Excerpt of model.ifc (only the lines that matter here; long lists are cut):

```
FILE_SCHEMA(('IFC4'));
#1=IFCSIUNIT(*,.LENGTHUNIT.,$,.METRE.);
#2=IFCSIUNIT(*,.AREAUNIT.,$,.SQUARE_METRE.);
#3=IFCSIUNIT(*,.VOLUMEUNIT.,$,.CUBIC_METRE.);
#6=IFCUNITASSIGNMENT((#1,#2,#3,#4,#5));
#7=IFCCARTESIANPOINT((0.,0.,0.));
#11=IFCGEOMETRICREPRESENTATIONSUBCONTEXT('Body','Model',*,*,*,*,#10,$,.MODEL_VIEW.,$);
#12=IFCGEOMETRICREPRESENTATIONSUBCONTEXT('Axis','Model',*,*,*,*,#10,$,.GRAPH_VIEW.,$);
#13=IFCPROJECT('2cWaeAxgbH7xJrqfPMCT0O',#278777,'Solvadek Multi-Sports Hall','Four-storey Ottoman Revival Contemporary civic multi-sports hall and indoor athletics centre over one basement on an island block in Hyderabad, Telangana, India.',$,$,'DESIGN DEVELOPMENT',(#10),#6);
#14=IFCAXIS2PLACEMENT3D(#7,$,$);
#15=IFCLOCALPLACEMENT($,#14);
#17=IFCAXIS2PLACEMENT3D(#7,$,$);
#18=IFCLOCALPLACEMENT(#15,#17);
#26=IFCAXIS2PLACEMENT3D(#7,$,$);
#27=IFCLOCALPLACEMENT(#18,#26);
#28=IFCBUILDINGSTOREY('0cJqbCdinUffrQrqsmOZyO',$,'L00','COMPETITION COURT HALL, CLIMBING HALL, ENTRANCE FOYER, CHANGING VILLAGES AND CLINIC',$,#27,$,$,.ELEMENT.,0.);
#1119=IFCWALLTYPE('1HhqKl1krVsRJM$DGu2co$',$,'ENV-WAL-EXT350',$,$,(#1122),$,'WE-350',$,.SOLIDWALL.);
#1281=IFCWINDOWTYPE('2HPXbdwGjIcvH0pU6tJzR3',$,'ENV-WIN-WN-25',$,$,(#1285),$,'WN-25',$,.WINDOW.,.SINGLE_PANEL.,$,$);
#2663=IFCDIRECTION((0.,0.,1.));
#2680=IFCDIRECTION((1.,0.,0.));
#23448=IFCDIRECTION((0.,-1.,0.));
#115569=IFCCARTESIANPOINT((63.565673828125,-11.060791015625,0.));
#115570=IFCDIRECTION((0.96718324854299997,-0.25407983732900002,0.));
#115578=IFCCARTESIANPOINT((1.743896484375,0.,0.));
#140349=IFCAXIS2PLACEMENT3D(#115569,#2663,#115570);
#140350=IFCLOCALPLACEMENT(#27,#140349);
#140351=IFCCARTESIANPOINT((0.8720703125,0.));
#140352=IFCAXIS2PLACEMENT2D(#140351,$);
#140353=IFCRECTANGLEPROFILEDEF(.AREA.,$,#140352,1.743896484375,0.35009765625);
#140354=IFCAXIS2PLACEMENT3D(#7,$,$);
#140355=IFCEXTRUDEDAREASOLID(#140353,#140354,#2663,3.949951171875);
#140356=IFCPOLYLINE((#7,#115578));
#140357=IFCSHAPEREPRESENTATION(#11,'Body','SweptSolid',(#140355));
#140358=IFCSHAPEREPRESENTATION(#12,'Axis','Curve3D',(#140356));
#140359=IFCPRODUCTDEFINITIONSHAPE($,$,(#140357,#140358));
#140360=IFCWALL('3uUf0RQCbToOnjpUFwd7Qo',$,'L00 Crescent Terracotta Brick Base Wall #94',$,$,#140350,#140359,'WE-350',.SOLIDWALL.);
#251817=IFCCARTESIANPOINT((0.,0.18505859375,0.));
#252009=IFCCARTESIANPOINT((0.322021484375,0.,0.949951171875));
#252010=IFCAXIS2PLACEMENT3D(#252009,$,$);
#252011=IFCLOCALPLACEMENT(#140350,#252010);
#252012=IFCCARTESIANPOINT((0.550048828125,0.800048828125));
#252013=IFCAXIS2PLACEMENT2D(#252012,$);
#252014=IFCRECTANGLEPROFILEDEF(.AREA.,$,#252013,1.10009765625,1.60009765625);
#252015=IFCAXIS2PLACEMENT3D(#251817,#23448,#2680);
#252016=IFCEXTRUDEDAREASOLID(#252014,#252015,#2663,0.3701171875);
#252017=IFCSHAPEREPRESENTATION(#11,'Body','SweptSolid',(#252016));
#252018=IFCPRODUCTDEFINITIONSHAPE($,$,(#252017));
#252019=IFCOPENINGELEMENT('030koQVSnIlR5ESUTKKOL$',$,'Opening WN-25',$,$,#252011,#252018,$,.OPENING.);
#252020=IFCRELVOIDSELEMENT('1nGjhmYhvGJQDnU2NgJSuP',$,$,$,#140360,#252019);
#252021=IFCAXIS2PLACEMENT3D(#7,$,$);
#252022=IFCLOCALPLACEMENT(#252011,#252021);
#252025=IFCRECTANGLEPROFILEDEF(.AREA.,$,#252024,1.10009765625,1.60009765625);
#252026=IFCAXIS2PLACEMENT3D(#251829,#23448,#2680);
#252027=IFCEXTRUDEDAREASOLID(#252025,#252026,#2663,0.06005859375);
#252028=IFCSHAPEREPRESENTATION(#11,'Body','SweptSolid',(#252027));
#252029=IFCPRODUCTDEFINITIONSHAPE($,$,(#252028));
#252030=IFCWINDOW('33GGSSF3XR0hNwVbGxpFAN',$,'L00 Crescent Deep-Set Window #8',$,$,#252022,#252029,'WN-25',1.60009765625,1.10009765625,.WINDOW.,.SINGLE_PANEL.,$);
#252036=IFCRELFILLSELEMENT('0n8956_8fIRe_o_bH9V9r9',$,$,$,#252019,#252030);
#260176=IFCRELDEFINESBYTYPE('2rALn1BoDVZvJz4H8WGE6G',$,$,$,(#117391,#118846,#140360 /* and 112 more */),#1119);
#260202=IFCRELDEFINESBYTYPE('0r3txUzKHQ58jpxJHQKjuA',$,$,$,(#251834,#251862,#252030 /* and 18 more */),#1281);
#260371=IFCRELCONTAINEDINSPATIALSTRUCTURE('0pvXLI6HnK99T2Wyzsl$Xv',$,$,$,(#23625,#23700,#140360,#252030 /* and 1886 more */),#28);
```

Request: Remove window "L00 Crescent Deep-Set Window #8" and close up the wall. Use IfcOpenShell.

```python
import ifcopenshell
import ifcopenshell.api.feature
import ifcopenshell.api.root
import ifcopenshell.geom
import ifcopenshell.util.shape

model = ifcopenshell.open("model.ifc")
settings = ifcopenshell.geom.settings()


def volume(element):
    """Net volume in cubic metres, openings subtracted."""
    shape = ifcopenshell.geom.create_shape(settings, element)
    return ifcopenshell.util.shape.get_volume(shape.geometry)


window = model.by_guid("33GGSSF3XR0hNwVbGxpFAN")
opening = window.FillsVoids[0].RelatingOpeningElement
wall = opening.VoidsElements[0].RelatingBuildingElement
before = volume(wall)

ifcopenshell.api.root.remove_product(model, product=window)
ifcopenshell.api.feature.remove_feature(model, feature=opening)

after = volume(wall)

print(f"wall volume {before:.3f} -> {after:.3f} m3")

model.write("model_updated.ifc")
```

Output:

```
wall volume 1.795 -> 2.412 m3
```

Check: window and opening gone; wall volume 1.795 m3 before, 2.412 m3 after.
